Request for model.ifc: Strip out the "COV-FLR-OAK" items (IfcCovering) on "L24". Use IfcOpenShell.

First a look at what the model holds.

```python
import ifcopenshell
import ifcopenshell.util.element

model = ifcopenshell.open("model.ifc")
print(model.schema)
storey = next(s for s in model.by_type("IfcBuildingStorey") if s.Name == "L24")
coverings = [e for e in ifcopenshell.util.element.get_decomposition(storey) if e.is_a("IfcCovering")]
seen = {}
for e in coverings:
    element_type = ifcopenshell.util.element.get_type(e)
    name = element_type.Name if element_type not in (None, e) else None
    seen[name] = seen.get(name, 0) + 1
for name, count in sorted(seen.items(), key=str):
    print(count, "x", name)
```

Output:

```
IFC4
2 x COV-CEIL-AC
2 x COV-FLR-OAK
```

```python
import ifcopenshell
import ifcopenshell.api.root
import ifcopenshell.util.element

model = ifcopenshell.open("model.ifc")

storey = next(s for s in model.by_type("IfcBuildingStorey") if s.Name == "L24")
coverings = [e for e in ifcopenshell.util.element.get_decomposition(storey) if e.is_a("IfcCovering")]
targets = [e for e in coverings if (t := ifcopenshell.util.element.get_type(e)) not in (None, e) and t.Name == "COV-FLR-OAK"]

for e in targets:
    ifcopenshell.api.root.remove_product(model, product=e)
print(len(targets), "removed")

model.write("model_edited.ifc")
```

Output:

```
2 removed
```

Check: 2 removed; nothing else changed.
